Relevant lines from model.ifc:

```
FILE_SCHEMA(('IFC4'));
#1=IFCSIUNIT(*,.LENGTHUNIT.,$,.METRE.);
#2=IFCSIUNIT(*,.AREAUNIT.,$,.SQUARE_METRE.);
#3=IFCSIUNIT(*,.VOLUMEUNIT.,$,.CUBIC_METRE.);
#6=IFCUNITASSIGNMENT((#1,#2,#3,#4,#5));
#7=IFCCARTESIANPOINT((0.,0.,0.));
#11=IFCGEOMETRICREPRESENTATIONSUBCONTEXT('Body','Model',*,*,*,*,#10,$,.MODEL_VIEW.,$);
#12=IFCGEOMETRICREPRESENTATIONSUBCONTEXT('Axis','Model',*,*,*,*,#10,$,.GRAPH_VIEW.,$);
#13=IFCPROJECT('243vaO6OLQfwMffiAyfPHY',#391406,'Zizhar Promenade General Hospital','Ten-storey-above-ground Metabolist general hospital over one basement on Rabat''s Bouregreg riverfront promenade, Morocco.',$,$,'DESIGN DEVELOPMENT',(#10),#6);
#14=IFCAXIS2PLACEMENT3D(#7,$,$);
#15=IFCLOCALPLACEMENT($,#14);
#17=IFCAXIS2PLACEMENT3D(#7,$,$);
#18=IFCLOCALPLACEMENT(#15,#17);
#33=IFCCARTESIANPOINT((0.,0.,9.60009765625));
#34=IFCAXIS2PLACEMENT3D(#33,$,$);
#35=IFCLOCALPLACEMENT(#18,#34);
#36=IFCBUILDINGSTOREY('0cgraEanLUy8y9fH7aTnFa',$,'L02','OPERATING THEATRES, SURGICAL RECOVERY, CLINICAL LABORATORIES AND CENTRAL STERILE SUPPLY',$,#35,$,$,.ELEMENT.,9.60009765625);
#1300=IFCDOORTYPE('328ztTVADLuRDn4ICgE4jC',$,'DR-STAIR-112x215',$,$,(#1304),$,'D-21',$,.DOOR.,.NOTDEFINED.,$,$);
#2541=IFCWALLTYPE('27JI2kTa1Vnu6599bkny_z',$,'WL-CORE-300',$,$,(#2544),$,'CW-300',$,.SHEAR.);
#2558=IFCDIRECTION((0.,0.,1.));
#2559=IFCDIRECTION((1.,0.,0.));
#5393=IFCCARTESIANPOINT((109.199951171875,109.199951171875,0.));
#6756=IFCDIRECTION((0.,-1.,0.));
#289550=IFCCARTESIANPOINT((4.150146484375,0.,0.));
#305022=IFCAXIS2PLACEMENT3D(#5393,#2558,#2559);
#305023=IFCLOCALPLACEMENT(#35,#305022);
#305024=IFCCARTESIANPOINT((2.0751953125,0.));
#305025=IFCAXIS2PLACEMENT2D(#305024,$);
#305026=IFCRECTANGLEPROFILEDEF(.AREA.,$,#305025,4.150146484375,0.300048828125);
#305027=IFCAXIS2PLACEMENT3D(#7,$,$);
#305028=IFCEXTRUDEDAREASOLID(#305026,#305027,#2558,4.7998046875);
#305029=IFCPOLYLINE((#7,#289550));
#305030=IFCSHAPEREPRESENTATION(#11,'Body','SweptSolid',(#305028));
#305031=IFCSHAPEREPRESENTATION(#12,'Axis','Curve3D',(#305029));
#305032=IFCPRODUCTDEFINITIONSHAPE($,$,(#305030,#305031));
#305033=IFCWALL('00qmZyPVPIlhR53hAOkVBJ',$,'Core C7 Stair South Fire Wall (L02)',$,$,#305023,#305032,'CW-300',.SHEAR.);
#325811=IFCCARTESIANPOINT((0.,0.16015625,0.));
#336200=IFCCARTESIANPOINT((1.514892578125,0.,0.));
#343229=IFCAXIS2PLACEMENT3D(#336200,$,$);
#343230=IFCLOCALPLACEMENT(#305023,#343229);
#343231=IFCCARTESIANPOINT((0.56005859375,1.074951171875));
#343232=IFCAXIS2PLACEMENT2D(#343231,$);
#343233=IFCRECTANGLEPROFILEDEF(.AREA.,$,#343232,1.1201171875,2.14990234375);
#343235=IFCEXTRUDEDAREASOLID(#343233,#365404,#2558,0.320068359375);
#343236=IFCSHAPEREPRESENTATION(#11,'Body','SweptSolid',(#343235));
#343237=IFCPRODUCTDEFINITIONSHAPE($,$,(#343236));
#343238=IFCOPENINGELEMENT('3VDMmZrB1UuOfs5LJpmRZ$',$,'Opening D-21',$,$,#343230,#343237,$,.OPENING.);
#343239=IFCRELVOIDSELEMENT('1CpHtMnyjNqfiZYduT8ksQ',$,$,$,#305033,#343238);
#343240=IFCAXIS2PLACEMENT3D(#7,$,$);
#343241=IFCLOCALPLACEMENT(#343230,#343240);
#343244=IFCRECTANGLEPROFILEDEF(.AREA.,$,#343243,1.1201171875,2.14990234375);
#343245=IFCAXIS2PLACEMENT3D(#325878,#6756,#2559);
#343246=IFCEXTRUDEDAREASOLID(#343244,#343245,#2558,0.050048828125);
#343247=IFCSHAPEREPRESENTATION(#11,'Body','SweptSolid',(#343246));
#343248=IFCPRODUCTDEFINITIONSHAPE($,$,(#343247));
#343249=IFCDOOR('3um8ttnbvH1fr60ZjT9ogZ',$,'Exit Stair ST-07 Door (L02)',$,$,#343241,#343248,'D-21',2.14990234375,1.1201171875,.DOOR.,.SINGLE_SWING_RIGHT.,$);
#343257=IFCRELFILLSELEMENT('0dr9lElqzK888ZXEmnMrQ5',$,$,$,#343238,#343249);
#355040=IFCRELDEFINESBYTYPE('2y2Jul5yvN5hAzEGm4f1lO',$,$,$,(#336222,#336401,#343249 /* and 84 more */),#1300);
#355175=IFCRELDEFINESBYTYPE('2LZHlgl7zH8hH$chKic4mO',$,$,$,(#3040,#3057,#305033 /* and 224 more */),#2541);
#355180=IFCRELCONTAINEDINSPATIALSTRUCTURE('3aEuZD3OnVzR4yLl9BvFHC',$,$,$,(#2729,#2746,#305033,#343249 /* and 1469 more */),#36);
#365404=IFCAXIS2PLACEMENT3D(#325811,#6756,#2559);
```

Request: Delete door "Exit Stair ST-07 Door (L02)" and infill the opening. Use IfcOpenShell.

```python
import ifcopenshell
import ifcopenshell.api.feature
import ifcopenshell.api.root
import ifcopenshell.geom
import ifcopenshell.util.shape

model = ifcopenshell.open("model.ifc")
settings = ifcopenshell.geom.settings()


def volume(element):
    """Net volume in cubic metres, openings subtracted."""
    shape = ifcopenshell.geom.create_shape(settings, element)
    return ifcopenshell.util.shape.get_volume(shape.geometry)


door = model.by_guid("3um8ttnbvH1fr60ZjT9ogZ")
opening = door.FillsVoids[0].RelatingOpeningElement
wall = opening.VoidsElements[0].RelatingBuildingElement
before = volume(wall)

ifcopenshell.api.root.remove_product(model, product=door)
ifcopenshell.api.feature.remove_feature(model, feature=opening)

after = volume(wall)

print(f"wall volume {before:.3f} -> {after:.3f} m3")

model.write("model_edited.ifc")
```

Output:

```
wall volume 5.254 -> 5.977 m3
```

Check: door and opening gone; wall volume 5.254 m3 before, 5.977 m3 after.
